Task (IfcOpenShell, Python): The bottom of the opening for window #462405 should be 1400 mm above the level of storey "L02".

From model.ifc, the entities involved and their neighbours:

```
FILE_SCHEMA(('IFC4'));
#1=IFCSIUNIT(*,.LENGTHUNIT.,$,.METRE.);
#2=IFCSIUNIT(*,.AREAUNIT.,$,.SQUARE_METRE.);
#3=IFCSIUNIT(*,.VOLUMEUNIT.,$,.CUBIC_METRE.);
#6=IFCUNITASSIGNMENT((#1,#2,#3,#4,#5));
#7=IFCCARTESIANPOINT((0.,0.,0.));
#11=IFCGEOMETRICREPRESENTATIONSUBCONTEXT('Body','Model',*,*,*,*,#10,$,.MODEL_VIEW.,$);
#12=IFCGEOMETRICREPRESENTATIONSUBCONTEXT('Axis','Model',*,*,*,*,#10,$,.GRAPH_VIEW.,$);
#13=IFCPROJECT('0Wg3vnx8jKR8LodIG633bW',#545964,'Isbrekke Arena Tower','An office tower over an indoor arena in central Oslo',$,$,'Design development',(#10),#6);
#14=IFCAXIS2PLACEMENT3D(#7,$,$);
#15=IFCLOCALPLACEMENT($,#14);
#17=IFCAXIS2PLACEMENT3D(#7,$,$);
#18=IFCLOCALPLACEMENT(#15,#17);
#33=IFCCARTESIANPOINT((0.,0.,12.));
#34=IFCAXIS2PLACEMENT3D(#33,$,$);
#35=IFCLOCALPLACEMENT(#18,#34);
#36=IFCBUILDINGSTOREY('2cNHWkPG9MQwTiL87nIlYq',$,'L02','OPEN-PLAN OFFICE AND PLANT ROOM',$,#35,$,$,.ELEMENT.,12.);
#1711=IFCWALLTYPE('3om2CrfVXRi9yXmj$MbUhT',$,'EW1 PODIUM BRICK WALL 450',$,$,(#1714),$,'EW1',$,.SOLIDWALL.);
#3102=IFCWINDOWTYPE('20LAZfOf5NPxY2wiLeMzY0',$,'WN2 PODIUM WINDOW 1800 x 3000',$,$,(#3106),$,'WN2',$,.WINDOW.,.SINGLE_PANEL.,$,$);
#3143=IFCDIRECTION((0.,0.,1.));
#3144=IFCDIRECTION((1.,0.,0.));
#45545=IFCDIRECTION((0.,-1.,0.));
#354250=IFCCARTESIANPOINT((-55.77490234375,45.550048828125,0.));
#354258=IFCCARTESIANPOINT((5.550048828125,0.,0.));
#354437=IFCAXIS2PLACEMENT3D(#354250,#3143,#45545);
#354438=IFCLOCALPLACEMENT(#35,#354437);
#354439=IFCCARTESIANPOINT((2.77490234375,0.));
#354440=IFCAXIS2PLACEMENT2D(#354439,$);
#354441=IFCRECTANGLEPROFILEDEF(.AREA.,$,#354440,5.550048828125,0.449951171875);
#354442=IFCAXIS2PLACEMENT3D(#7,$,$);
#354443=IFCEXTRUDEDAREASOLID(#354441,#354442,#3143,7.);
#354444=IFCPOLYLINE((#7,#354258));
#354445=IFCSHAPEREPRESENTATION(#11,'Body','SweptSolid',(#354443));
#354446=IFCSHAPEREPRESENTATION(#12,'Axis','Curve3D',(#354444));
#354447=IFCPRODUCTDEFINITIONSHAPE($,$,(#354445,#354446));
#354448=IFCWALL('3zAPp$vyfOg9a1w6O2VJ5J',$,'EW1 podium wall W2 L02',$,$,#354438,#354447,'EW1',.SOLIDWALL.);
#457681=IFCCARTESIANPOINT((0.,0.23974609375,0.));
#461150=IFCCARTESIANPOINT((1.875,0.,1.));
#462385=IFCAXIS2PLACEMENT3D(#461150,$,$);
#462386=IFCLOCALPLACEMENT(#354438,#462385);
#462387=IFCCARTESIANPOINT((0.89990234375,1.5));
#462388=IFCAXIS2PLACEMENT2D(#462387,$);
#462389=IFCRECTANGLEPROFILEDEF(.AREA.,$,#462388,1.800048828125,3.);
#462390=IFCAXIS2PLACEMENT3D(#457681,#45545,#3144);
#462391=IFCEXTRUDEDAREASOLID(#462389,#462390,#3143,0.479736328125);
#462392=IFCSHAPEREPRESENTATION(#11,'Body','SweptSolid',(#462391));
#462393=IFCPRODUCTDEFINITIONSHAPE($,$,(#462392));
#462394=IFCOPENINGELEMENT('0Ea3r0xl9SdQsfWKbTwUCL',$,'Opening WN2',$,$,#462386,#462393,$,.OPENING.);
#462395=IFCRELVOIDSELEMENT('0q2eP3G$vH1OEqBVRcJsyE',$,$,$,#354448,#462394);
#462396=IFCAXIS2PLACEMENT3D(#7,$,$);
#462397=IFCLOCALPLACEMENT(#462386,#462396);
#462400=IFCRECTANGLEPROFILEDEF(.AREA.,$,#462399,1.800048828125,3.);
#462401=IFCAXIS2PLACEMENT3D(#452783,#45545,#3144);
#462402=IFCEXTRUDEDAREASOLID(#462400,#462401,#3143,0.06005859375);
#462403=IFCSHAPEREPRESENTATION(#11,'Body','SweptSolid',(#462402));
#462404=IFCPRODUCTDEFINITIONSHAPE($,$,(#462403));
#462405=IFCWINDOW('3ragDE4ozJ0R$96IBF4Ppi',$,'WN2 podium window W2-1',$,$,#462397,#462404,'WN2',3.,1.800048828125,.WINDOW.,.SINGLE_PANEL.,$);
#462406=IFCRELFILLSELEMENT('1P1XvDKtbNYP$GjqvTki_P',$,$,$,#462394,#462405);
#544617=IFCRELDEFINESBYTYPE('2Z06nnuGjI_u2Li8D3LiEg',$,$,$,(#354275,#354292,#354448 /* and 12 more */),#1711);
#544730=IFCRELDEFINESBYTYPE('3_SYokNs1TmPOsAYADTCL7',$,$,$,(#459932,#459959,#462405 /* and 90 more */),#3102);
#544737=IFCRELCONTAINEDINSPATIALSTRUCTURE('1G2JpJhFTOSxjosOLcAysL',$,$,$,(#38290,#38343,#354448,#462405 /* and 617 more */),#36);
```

```python
import numpy as np
import ifcopenshell
import ifcopenshell.api.geometry
import ifcopenshell.geom
import ifcopenshell.util.element
import ifcopenshell.util.placement
import ifcopenshell.util.shape
import ifcopenshell.util.unit

model = ifcopenshell.open("model.ifc")
unit_scale = ifcopenshell.util.unit.calculate_unit_scale(model)

window = model.by_guid("3ragDE4ozJ0R$96IBF4Ppi")
opening = window.FillsVoids[0].RelatingOpeningElement
storey = ifcopenshell.util.element.get_container(window, ifc_class="IfcBuildingStorey")
level = ifcopenshell.util.placement.get_local_placement(storey.ObjectPlacement)[2, 3]

# The opening's origin need not be at the sill, so measure its lowest point.
shape = ifcopenshell.geom.create_shape(ifcopenshell.geom.settings(), opening)
bottom = ifcopenshell.util.shape.get_shape_bottom_elevation(shape, shape.geometry) / unit_scale
dz = level + 1.4 / unit_scale - bottom

shift = np.array([0.0, 0.0, dz])
# The window is placed relative to its opening, so it follows when the opening moves.
matrix = ifcopenshell.util.placement.get_local_placement(opening.ObjectPlacement)
matrix[:3, 3] += shift
ifcopenshell.api.geometry.edit_object_placement(
    model, product=opening, matrix=matrix, is_si=False, should_transform_children=True
)

print(f"moved by {dz * unit_scale:+.3f} m")

model.write("model_updated.ifc")
```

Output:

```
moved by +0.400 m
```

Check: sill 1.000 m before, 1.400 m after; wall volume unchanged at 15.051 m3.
